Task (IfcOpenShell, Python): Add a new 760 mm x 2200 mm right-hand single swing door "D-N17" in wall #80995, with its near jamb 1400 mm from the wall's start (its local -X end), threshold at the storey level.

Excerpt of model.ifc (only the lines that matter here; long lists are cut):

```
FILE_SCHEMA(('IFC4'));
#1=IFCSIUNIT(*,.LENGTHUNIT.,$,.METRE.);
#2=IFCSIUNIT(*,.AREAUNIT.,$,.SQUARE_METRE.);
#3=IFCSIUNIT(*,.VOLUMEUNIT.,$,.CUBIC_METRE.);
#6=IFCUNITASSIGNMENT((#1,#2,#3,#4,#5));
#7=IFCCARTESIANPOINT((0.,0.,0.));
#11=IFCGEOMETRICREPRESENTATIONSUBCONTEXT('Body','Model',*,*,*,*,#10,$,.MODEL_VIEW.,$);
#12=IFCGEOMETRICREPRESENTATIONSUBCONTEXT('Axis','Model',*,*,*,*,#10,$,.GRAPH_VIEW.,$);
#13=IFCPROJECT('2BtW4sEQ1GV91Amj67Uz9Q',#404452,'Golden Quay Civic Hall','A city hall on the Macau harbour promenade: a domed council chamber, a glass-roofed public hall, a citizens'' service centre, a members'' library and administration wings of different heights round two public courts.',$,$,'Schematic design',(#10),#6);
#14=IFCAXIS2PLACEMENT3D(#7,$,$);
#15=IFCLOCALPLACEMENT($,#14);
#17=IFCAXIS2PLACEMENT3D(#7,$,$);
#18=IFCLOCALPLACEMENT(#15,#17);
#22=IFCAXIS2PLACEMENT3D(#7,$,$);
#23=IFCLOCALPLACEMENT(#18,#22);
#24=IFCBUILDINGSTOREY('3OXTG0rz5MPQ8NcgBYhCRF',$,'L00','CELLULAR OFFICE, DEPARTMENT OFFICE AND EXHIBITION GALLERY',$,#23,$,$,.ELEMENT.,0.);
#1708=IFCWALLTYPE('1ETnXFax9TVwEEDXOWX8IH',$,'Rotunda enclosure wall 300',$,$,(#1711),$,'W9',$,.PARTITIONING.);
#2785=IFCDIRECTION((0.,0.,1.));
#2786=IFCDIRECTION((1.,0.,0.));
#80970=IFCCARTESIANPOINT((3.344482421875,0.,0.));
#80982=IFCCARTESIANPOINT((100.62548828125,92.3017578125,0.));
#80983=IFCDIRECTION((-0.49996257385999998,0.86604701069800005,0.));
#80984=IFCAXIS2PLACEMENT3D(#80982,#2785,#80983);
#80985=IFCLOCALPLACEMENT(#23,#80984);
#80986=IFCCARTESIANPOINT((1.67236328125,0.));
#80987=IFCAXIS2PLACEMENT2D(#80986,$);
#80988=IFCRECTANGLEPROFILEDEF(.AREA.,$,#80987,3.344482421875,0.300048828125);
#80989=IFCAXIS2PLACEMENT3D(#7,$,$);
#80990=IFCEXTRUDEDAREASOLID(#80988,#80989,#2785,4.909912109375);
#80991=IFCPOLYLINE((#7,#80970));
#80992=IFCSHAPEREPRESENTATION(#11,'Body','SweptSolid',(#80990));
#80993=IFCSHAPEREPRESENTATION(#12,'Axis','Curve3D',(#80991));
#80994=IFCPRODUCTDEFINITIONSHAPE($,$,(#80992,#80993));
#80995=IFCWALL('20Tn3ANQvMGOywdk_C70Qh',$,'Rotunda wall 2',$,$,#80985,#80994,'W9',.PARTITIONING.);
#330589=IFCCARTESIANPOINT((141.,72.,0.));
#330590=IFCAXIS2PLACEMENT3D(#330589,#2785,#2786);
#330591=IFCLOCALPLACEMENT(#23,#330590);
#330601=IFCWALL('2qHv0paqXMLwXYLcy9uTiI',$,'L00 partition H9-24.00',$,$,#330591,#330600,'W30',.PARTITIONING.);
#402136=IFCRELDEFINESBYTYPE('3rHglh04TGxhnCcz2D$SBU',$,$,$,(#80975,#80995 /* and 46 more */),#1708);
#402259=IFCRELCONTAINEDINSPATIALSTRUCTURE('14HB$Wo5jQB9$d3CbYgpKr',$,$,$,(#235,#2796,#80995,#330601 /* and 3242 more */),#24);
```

```python
import numpy as np
import ifcopenshell
import ifcopenshell.api.feature
import ifcopenshell.api.geometry
import ifcopenshell.api.root
import ifcopenshell.api.spatial
import ifcopenshell.geom
import ifcopenshell.util.element
import ifcopenshell.util.placement
import ifcopenshell.util.representation
import ifcopenshell.util.shape
import ifcopenshell.util.unit

model = ifcopenshell.open("model.ifc")
unit_scale = ifcopenshell.util.unit.calculate_unit_scale(model)
settings = ifcopenshell.geom.settings()


def volume(element):
    """Net volume in cubic metres, openings subtracted."""
    shape = ifcopenshell.geom.create_shape(settings, element)
    return ifcopenshell.util.shape.get_volume(shape.geometry)


wall = model.by_id(80995)
storey = ifcopenshell.util.element.get_container(wall, ifc_class="IfcBuildingStorey")
context = ifcopenshell.util.representation.get_context(model, "Model", "Body", "MODEL_VIEW")
before = volume(wall)

width, height, from_end, sill = 0.76, 2.2, 1.4, 0.0  # metres

# The wall runs along its own X axis, and the end named is its -X end.
wall_shape = ifcopenshell.geom.create_shape(settings, wall)
x, y, z = ifcopenshell.util.shape.get_vertices(wall_shape.geometry).T
start = x.min() + from_end
face, thickness = float(y.min()), float(y.max() - y.min())
wall_matrix = ifcopenshell.util.placement.get_local_placement(wall.ObjectPlacement)
level = ifcopenshell.util.placement.get_local_placement(storey.ObjectPlacement)[2, 3]


def in_wall(x, y):
    """Placement at x, y metres in the wall's axes, at sill height."""
    matrix = wall_matrix.copy()
    matrix[:, 3] = wall_matrix @ np.array([x / unit_scale, y / unit_scale, 0.0, 1.0])
    matrix[2, 3] = level + sill / unit_scale
    return matrix


# Opening: a box that overshoots both wall faces by 50 mm.
opening = ifcopenshell.api.root.create_entity(model, ifc_class="IfcOpeningElement", predefined_type="OPENING")
box = ifcopenshell.api.geometry.add_wall_representation(
    model, context=context, length=width, height=height, thickness=thickness + 0.1
)
ifcopenshell.api.geometry.assign_representation(model, product=opening, representation=box)
ifcopenshell.api.geometry.edit_object_placement(model, product=opening, matrix=in_wall(start, face - 0.05), is_si=False)
ifcopenshell.api.feature.add_feature(model, feature=opening, element=wall)

door = ifcopenshell.api.root.create_entity(model, ifc_class="IfcDoor", name="D-N17", predefined_type="DOOR")
door.OverallWidth, door.OverallHeight = width / unit_scale, height / unit_scale
door.OperationType = "SINGLE_SWING_RIGHT"
body = ifcopenshell.api.geometry.add_door_representation(
    model,
    context=context,
    overall_width=door.OverallWidth,
    overall_height=door.OverallHeight,
    operation_type="SINGLE_SWING_RIGHT",
    lining_properties={"LiningDepth": thickness / unit_scale, "ThresholdDepth": thickness / unit_scale},
)
ifcopenshell.api.geometry.assign_representation(model, product=door, representation=body)
ifcopenshell.api.spatial.assign_container(model, products=[door], relating_structure=storey)
ifcopenshell.api.feature.add_filling(model, opening=opening, element=door)

# The lining spans the wall, so the door starts at the wall face.
ifcopenshell.api.geometry.edit_object_placement(model, product=door, matrix=in_wall(start, face), is_si=False)

after = volume(wall)

print(f"wall volume {before:.3f} -> {after:.3f} m3")

model.write("model_edited.ifc")
```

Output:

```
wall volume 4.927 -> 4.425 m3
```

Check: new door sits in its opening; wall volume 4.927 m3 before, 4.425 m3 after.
